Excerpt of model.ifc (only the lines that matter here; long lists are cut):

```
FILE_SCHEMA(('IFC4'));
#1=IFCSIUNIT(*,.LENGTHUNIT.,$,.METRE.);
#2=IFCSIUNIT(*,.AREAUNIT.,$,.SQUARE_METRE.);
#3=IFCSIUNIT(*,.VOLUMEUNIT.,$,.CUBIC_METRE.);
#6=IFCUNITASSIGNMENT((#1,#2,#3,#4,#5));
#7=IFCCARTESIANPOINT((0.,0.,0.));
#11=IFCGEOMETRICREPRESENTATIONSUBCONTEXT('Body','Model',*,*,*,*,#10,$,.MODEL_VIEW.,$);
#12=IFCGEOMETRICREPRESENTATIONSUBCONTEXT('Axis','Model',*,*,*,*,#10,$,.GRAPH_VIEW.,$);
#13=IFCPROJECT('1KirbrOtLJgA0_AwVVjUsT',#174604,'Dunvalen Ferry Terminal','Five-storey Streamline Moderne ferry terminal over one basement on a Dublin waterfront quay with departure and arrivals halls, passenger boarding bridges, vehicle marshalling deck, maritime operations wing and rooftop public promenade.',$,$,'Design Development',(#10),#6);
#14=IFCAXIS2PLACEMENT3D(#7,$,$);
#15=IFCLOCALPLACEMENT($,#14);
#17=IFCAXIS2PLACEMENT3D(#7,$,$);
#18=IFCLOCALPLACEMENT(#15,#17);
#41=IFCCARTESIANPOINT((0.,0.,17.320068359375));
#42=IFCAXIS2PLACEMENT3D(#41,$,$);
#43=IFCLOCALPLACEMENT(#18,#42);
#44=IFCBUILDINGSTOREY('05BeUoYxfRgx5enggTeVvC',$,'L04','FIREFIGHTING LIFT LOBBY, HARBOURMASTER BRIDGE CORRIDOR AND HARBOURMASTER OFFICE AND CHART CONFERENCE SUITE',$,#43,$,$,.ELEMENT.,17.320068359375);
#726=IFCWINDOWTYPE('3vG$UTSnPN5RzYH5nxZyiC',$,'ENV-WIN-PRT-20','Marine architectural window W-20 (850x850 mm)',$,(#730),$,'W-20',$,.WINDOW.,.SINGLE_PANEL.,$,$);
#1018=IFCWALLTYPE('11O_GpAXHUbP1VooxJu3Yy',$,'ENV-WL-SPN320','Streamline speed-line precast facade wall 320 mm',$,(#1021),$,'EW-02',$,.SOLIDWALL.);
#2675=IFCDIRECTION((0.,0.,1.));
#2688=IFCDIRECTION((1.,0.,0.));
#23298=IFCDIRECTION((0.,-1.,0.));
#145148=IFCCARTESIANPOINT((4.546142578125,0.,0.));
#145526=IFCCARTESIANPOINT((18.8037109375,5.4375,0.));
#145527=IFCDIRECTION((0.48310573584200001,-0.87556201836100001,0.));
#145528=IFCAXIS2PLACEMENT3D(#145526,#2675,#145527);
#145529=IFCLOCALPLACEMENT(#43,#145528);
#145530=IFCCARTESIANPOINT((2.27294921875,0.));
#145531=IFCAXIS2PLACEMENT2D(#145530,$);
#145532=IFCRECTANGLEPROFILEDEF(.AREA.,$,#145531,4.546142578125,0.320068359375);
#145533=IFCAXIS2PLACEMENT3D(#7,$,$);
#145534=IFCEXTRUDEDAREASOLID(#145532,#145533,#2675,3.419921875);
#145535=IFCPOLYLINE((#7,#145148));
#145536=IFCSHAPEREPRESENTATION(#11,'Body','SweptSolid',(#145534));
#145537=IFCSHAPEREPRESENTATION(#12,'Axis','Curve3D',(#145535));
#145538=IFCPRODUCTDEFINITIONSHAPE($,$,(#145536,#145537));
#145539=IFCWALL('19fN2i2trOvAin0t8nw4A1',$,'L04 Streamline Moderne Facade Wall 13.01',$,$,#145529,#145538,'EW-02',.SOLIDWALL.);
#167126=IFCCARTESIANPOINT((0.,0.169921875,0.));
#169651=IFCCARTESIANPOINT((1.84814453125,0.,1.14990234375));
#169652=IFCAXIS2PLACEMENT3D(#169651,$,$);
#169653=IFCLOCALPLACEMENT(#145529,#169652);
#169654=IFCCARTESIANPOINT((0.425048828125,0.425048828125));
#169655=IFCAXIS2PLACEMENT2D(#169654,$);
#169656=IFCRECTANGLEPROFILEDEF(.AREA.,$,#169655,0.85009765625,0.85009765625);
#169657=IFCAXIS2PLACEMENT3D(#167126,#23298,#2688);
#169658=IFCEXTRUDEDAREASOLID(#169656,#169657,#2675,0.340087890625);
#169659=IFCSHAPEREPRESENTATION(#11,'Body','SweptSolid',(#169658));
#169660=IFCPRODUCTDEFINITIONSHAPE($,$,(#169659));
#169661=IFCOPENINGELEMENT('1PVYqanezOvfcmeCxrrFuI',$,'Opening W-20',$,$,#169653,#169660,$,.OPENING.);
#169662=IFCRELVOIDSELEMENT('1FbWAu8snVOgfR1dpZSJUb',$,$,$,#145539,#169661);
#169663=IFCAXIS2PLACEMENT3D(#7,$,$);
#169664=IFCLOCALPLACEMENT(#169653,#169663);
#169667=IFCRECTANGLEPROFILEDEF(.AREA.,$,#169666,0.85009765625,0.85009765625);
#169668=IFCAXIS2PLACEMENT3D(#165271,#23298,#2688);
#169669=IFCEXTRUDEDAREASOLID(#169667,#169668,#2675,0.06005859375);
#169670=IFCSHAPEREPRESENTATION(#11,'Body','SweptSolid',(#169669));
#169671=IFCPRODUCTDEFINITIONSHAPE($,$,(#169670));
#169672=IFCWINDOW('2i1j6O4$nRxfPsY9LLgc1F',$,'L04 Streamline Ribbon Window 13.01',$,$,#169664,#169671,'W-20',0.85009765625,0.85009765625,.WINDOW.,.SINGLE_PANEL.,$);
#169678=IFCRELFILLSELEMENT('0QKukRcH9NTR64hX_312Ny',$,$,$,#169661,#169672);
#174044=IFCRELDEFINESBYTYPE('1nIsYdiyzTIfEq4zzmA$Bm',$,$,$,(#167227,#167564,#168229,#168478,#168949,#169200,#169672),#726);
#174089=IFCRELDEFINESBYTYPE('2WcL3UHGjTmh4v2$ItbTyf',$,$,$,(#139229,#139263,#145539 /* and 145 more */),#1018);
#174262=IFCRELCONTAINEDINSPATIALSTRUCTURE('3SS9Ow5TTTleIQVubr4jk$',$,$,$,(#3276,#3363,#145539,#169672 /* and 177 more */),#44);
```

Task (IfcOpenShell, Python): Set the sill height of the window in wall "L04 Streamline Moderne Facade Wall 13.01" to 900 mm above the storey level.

```python
import numpy as np
import ifcopenshell
import ifcopenshell.api.geometry
import ifcopenshell.geom
import ifcopenshell.util.element
import ifcopenshell.util.placement
import ifcopenshell.util.shape
import ifcopenshell.util.unit

model = ifcopenshell.open("model.ifc")
unit_scale = ifcopenshell.util.unit.calculate_unit_scale(model)

window = model.by_guid("2i1j6O4$nRxfPsY9LLgc1F")
opening = window.FillsVoids[0].RelatingOpeningElement
storey = ifcopenshell.util.element.get_container(window, ifc_class="IfcBuildingStorey")
level = ifcopenshell.util.placement.get_local_placement(storey.ObjectPlacement)[2, 3]

# The opening's origin need not be at the sill, so measure its lowest point.
shape = ifcopenshell.geom.create_shape(ifcopenshell.geom.settings(), opening)
bottom = ifcopenshell.util.shape.get_shape_bottom_elevation(shape, shape.geometry) / unit_scale
dz = level + 0.9 / unit_scale - bottom

shift = np.array([0.0, 0.0, dz])
# The window is placed relative to its opening, so it follows when the opening moves.
matrix = ifcopenshell.util.placement.get_local_placement(opening.ObjectPlacement)
matrix[:3, 3] += shift
ifcopenshell.api.geometry.edit_object_placement(
    model, product=opening, matrix=matrix, is_si=False, should_transform_children=True
)

print(f"moved by {dz * unit_scale:+.3f} m")

model.write("model_v2.ifc")
```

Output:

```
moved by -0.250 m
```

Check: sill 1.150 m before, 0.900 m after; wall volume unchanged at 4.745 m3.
